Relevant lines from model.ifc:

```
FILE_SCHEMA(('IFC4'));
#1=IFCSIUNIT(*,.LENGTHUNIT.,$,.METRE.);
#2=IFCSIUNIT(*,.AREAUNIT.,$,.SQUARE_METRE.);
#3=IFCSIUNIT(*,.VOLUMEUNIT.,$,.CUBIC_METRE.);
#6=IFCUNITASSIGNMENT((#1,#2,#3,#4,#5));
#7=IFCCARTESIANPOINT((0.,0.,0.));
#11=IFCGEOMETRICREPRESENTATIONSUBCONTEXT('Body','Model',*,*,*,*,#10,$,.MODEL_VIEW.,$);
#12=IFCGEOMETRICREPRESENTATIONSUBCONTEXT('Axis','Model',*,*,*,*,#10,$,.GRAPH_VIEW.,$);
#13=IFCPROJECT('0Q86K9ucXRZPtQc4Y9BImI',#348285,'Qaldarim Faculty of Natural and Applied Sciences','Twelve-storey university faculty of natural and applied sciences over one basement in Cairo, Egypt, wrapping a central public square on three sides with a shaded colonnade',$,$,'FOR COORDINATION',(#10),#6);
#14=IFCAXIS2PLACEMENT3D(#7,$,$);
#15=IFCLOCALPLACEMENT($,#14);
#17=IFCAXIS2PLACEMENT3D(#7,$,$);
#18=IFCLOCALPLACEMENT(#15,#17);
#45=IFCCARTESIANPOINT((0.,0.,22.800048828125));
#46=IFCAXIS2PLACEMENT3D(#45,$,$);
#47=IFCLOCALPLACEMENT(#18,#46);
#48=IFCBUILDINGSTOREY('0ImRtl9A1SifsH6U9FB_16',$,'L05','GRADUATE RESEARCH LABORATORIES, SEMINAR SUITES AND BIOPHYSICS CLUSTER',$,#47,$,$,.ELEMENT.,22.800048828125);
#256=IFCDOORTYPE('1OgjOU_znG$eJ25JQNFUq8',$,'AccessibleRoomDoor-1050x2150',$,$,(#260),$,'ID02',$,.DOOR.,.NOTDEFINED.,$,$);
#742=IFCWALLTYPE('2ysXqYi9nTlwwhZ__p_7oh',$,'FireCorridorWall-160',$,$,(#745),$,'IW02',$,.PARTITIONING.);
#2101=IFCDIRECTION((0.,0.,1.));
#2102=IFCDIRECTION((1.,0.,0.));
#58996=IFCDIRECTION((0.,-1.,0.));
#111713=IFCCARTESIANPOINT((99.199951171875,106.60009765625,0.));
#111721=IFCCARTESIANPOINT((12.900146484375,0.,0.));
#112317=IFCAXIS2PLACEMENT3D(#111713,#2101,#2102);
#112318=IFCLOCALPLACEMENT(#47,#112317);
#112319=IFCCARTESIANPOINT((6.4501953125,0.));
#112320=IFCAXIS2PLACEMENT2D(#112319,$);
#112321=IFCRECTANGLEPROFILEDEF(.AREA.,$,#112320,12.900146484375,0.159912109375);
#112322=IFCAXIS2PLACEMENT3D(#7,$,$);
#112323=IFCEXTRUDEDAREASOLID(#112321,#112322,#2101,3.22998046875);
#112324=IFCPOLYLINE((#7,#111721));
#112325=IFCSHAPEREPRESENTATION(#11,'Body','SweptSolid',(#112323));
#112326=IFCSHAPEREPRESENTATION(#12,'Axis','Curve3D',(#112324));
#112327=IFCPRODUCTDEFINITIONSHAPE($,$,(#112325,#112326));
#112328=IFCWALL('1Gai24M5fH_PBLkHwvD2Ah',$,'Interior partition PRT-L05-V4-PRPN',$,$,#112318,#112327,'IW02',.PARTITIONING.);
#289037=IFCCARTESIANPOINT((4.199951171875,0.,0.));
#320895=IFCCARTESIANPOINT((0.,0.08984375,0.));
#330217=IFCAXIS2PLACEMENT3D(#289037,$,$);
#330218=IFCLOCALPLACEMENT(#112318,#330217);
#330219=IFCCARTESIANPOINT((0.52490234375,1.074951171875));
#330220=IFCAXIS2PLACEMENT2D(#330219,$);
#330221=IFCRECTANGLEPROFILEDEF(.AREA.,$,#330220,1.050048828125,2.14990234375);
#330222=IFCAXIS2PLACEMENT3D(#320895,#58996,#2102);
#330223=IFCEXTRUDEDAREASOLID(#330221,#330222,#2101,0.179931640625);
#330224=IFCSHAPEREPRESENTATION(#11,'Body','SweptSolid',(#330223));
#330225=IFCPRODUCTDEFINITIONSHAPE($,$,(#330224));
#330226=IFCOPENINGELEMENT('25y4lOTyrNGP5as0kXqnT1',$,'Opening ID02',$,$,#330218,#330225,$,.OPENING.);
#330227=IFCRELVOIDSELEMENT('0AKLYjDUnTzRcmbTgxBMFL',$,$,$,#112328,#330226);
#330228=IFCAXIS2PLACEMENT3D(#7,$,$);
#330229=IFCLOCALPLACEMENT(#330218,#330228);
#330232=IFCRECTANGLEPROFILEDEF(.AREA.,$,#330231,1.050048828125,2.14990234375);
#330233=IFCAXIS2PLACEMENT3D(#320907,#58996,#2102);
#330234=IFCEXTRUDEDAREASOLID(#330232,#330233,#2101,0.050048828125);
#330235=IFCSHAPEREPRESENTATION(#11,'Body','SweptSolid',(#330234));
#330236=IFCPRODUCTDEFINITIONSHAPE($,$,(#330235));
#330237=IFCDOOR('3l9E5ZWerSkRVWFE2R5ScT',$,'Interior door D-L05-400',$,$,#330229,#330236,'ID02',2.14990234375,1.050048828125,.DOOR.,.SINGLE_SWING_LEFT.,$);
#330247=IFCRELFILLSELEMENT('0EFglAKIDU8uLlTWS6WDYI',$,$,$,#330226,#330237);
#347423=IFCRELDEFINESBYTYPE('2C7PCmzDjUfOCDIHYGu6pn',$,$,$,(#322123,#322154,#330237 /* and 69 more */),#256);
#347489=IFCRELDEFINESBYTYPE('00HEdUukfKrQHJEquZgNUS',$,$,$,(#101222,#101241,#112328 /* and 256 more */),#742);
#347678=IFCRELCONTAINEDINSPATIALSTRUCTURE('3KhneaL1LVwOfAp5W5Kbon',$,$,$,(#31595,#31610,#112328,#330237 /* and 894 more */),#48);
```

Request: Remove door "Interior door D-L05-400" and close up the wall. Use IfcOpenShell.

```python
import ifcopenshell
import ifcopenshell.api.feature
import ifcopenshell.api.root
import ifcopenshell.geom
import ifcopenshell.util.shape

model = ifcopenshell.open("model.ifc")
settings = ifcopenshell.geom.settings()


def volume(element):
    """Net volume in cubic metres, openings subtracted."""
    shape = ifcopenshell.geom.create_shape(settings, element)
    return ifcopenshell.util.shape.get_volume(shape.geometry)


door = model.by_guid("3l9E5ZWerSkRVWFE2R5ScT")
opening = door.FillsVoids[0].RelatingOpeningElement
wall = opening.VoidsElements[0].RelatingBuildingElement
before = volume(wall)

ifcopenshell.api.root.remove_product(model, product=door)
ifcopenshell.api.feature.remove_feature(model, feature=opening)

after = volume(wall)

print(f"wall volume {before:.3f} -> {after:.3f} m3")

model.write("model_updated.ifc")
```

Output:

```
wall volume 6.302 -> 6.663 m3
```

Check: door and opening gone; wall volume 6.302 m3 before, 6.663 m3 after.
